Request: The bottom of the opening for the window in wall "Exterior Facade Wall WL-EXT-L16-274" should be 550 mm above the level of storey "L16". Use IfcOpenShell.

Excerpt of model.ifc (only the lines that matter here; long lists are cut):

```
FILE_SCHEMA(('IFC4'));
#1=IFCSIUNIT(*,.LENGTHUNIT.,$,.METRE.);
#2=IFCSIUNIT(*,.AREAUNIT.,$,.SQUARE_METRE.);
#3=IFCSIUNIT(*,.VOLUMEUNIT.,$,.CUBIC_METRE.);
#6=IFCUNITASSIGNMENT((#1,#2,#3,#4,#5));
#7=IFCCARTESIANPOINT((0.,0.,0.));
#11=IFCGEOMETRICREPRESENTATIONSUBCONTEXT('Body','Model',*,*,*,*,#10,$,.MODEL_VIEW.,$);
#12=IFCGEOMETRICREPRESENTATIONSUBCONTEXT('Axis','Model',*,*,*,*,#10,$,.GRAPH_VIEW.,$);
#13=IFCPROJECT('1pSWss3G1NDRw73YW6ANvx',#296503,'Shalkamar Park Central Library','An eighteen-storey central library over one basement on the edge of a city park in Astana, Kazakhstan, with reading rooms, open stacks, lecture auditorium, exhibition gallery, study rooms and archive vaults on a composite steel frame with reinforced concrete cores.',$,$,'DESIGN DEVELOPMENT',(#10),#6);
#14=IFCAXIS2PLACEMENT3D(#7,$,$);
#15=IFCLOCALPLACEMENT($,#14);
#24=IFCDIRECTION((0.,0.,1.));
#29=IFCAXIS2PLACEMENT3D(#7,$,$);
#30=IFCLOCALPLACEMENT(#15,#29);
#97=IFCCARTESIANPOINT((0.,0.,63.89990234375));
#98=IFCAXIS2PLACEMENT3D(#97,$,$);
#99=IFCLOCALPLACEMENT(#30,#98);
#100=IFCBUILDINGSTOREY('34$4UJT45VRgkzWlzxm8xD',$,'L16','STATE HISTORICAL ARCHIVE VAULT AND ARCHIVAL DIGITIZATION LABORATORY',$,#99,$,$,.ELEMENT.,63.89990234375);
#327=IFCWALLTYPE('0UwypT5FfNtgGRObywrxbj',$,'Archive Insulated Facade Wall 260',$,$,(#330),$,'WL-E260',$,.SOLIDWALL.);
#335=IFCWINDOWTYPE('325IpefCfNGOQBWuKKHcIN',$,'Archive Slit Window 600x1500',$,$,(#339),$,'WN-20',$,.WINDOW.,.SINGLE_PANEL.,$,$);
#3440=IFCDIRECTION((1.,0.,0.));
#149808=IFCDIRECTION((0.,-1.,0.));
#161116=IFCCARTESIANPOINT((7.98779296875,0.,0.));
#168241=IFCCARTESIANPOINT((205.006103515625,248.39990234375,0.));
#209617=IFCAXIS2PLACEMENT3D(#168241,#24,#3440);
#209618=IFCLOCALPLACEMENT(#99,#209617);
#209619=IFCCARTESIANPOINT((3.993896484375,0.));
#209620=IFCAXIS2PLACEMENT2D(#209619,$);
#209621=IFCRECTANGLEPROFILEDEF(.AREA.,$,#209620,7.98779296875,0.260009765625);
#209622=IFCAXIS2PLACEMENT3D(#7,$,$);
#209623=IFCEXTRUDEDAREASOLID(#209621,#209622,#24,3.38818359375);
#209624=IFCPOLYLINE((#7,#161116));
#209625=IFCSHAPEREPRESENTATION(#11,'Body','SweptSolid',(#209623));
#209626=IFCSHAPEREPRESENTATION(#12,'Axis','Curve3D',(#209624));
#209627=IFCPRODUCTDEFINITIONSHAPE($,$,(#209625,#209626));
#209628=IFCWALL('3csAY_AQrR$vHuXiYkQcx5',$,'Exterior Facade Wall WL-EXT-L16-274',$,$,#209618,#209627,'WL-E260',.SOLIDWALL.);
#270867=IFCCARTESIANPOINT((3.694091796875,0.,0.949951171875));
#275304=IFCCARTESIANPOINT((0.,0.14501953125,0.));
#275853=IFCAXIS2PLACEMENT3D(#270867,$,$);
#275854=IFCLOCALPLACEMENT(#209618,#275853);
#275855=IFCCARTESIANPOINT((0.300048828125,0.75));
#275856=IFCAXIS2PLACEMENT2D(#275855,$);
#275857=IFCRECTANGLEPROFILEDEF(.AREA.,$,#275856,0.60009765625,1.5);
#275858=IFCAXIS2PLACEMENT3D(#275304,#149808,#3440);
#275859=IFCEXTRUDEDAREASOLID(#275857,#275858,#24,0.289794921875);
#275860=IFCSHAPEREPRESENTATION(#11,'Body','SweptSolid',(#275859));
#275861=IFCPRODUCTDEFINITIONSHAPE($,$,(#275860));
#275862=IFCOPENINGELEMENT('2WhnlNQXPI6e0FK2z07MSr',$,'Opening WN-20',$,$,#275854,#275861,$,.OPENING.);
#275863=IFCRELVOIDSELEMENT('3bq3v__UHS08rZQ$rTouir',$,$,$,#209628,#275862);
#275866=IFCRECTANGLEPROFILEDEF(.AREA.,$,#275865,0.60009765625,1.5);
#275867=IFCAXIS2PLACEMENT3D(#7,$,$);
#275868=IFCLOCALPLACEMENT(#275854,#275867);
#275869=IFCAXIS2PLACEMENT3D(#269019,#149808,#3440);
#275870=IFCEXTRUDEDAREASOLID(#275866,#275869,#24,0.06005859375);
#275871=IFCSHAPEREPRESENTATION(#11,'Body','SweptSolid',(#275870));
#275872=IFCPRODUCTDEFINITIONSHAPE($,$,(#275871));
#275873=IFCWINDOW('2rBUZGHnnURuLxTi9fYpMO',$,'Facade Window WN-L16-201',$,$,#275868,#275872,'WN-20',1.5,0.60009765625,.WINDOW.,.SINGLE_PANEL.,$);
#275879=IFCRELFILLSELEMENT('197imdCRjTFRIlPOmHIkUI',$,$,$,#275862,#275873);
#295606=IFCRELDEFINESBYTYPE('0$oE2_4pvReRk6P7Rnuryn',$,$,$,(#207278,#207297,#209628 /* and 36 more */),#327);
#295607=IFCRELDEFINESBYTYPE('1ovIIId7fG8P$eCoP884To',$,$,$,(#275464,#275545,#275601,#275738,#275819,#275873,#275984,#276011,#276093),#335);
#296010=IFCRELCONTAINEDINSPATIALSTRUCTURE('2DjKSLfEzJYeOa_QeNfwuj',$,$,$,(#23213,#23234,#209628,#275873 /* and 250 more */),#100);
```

```python
import numpy as np
import ifcopenshell
import ifcopenshell.api.geometry
import ifcopenshell.geom
import ifcopenshell.util.element
import ifcopenshell.util.placement
import ifcopenshell.util.shape
import ifcopenshell.util.unit

model = ifcopenshell.open("model.ifc")
unit_scale = ifcopenshell.util.unit.calculate_unit_scale(model)

window = model.by_guid("2rBUZGHnnURuLxTi9fYpMO")
opening = window.FillsVoids[0].RelatingOpeningElement
storey = ifcopenshell.util.element.get_container(window, ifc_class="IfcBuildingStorey")
level = ifcopenshell.util.placement.get_local_placement(storey.ObjectPlacement)[2, 3]

# The opening's origin need not be at the sill, so measure its lowest point.
shape = ifcopenshell.geom.create_shape(ifcopenshell.geom.settings(), opening)
bottom = ifcopenshell.util.shape.get_shape_bottom_elevation(shape, shape.geometry) / unit_scale
dz = level + 0.55 - bottom

shift = np.array([0.0, 0.0, dz])
# The window is placed relative to its opening, so it follows when the opening moves.
matrix = ifcopenshell.util.placement.get_local_placement(opening.ObjectPlacement)
matrix[:3, 3] += shift
ifcopenshell.api.geometry.edit_object_placement(
    model, product=opening, matrix=matrix, is_si=False, should_transform_children=True
)

print(f"moved by {dz * unit_scale:+.3f} m")

model.write("model_edited.ifc")
```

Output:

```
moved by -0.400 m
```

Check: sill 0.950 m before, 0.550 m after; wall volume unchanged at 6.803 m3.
